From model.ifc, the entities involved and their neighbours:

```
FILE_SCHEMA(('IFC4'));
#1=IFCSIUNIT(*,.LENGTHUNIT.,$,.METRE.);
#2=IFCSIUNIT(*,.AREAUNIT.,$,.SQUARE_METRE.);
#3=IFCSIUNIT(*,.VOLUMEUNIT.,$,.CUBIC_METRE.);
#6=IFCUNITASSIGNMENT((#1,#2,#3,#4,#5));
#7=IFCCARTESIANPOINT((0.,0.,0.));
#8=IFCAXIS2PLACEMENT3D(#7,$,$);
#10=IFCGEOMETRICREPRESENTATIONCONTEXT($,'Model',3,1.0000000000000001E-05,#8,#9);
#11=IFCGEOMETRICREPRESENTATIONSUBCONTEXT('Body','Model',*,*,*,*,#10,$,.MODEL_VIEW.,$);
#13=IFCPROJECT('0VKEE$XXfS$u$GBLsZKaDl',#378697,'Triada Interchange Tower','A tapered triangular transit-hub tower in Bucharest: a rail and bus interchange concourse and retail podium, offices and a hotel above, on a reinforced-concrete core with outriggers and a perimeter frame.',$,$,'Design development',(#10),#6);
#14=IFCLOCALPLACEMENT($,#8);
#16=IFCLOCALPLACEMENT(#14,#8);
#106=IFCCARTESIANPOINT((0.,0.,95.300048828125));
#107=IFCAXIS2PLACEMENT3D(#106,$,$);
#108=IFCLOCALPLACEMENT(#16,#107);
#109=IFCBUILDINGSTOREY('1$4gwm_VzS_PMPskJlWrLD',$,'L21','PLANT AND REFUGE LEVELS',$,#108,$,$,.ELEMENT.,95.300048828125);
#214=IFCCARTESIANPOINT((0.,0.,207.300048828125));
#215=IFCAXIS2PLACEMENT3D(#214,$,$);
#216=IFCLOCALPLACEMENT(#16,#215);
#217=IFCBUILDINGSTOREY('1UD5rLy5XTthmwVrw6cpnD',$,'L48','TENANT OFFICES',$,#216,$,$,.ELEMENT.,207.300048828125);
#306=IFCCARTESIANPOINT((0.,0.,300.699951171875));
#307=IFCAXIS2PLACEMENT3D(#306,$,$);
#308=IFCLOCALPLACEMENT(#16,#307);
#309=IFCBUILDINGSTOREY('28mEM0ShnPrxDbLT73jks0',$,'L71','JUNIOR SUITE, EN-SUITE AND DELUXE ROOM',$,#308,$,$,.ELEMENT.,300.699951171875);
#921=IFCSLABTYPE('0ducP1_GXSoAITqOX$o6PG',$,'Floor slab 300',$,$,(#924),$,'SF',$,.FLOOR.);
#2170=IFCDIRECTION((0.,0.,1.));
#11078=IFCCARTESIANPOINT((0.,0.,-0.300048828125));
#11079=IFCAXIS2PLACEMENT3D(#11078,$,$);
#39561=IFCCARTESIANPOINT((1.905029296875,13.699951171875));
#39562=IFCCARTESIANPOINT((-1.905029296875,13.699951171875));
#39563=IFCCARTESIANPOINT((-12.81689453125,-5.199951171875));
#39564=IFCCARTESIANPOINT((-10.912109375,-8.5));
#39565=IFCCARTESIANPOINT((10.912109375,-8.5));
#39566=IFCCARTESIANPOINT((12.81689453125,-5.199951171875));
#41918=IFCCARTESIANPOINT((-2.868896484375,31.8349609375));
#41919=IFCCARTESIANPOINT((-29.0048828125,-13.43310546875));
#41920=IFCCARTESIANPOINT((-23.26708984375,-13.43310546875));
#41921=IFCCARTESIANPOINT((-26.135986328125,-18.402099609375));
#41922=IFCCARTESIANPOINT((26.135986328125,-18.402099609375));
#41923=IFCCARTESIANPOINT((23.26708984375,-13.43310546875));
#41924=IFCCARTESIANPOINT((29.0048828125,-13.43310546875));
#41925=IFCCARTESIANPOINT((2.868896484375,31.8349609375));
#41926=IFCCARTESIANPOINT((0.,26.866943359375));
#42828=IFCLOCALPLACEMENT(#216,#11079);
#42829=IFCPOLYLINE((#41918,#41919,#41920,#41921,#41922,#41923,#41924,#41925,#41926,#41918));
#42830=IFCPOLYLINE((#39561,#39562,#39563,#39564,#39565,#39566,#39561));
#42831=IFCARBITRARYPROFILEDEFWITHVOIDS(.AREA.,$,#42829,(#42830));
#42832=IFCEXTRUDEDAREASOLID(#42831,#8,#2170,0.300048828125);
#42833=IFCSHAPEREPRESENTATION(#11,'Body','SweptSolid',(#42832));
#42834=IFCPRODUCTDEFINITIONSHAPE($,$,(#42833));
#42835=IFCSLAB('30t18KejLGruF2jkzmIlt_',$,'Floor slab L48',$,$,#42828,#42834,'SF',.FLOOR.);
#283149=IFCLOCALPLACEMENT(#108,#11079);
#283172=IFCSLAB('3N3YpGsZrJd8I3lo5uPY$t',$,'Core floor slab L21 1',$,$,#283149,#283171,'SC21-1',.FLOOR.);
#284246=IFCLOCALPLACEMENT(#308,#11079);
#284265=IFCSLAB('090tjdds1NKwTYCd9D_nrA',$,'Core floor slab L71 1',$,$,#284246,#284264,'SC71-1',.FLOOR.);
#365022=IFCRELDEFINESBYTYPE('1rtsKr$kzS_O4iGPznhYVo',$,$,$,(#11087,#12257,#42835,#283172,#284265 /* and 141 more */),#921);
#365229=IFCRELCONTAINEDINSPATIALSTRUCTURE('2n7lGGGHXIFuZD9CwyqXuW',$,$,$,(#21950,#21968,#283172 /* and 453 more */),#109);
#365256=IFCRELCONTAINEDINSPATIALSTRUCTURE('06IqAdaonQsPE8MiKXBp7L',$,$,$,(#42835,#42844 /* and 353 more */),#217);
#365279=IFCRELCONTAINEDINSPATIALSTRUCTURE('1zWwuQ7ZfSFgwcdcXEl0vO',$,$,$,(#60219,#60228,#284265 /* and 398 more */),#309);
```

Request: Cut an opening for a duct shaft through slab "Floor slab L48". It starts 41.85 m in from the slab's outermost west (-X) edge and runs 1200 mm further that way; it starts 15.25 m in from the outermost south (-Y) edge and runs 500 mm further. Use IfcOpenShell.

```python
import numpy as np
import ifcopenshell
import ifcopenshell.api.feature
import ifcopenshell.api.geometry
import ifcopenshell.api.root
import ifcopenshell.geom
import ifcopenshell.util.placement
import ifcopenshell.util.representation
import ifcopenshell.util.shape
import ifcopenshell.util.unit

model = ifcopenshell.open("model.ifc")
unit_scale = ifcopenshell.util.unit.calculate_unit_scale(model)
settings = ifcopenshell.geom.settings()


def volume(element):
    """Net volume in cubic metres, openings subtracted."""
    shape = ifcopenshell.geom.create_shape(settings, element)
    return ifcopenshell.util.shape.get_volume(shape.geometry)


slab = model.by_guid("30t18KejLGruF2jkzmIlt_")
before = volume(slab)

# Extent in the slab's own axes, in metres. The edges named are its -X and -Y sides.
slab_shape = ifcopenshell.geom.create_shape(settings, slab)
vertices = ifcopenshell.util.shape.get_vertices(slab_shape.geometry)
x_min, y_min, bottom = vertices.min(axis=0)
top = vertices[:, 2].max()

opening = ifcopenshell.api.root.create_entity(model, ifc_class="IfcOpeningElement", name="Duct shaft opening", predefined_type="OPENING")
context = ifcopenshell.util.representation.get_context(model, "Model", "Body", "MODEL_VIEW")
width, depth = 1.2, 0.5
outline = [(0.0, 0.0), (width, 0.0), (width, depth), (0.0, depth), (0.0, 0.0)]
# Overshoot both faces by 50 mm so the cut is clean.
shape = ifcopenshell.api.geometry.add_slab_representation(
    model, context=context, depth=top - bottom + 0.1, polyline=outline
)
ifcopenshell.api.geometry.assign_representation(model, product=opening, representation=shape)

matrix = ifcopenshell.util.placement.get_local_placement(slab.ObjectPlacement)
matrix[:, 3] = matrix @ np.append(np.array([x_min + 41.85, y_min + 15.25, bottom - 0.05]) / unit_scale, 1.0)
ifcopenshell.api.geometry.edit_object_placement(model, product=opening, matrix=matrix, is_si=False)
ifcopenshell.api.feature.add_feature(model, feature=opening, element=slab)

after = volume(slab)

print(f"slab volume {before:.3f} -> {after:.3f} m3")

model.write("model_edited.ifc")
```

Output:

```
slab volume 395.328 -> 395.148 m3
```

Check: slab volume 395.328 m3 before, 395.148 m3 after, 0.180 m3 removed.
